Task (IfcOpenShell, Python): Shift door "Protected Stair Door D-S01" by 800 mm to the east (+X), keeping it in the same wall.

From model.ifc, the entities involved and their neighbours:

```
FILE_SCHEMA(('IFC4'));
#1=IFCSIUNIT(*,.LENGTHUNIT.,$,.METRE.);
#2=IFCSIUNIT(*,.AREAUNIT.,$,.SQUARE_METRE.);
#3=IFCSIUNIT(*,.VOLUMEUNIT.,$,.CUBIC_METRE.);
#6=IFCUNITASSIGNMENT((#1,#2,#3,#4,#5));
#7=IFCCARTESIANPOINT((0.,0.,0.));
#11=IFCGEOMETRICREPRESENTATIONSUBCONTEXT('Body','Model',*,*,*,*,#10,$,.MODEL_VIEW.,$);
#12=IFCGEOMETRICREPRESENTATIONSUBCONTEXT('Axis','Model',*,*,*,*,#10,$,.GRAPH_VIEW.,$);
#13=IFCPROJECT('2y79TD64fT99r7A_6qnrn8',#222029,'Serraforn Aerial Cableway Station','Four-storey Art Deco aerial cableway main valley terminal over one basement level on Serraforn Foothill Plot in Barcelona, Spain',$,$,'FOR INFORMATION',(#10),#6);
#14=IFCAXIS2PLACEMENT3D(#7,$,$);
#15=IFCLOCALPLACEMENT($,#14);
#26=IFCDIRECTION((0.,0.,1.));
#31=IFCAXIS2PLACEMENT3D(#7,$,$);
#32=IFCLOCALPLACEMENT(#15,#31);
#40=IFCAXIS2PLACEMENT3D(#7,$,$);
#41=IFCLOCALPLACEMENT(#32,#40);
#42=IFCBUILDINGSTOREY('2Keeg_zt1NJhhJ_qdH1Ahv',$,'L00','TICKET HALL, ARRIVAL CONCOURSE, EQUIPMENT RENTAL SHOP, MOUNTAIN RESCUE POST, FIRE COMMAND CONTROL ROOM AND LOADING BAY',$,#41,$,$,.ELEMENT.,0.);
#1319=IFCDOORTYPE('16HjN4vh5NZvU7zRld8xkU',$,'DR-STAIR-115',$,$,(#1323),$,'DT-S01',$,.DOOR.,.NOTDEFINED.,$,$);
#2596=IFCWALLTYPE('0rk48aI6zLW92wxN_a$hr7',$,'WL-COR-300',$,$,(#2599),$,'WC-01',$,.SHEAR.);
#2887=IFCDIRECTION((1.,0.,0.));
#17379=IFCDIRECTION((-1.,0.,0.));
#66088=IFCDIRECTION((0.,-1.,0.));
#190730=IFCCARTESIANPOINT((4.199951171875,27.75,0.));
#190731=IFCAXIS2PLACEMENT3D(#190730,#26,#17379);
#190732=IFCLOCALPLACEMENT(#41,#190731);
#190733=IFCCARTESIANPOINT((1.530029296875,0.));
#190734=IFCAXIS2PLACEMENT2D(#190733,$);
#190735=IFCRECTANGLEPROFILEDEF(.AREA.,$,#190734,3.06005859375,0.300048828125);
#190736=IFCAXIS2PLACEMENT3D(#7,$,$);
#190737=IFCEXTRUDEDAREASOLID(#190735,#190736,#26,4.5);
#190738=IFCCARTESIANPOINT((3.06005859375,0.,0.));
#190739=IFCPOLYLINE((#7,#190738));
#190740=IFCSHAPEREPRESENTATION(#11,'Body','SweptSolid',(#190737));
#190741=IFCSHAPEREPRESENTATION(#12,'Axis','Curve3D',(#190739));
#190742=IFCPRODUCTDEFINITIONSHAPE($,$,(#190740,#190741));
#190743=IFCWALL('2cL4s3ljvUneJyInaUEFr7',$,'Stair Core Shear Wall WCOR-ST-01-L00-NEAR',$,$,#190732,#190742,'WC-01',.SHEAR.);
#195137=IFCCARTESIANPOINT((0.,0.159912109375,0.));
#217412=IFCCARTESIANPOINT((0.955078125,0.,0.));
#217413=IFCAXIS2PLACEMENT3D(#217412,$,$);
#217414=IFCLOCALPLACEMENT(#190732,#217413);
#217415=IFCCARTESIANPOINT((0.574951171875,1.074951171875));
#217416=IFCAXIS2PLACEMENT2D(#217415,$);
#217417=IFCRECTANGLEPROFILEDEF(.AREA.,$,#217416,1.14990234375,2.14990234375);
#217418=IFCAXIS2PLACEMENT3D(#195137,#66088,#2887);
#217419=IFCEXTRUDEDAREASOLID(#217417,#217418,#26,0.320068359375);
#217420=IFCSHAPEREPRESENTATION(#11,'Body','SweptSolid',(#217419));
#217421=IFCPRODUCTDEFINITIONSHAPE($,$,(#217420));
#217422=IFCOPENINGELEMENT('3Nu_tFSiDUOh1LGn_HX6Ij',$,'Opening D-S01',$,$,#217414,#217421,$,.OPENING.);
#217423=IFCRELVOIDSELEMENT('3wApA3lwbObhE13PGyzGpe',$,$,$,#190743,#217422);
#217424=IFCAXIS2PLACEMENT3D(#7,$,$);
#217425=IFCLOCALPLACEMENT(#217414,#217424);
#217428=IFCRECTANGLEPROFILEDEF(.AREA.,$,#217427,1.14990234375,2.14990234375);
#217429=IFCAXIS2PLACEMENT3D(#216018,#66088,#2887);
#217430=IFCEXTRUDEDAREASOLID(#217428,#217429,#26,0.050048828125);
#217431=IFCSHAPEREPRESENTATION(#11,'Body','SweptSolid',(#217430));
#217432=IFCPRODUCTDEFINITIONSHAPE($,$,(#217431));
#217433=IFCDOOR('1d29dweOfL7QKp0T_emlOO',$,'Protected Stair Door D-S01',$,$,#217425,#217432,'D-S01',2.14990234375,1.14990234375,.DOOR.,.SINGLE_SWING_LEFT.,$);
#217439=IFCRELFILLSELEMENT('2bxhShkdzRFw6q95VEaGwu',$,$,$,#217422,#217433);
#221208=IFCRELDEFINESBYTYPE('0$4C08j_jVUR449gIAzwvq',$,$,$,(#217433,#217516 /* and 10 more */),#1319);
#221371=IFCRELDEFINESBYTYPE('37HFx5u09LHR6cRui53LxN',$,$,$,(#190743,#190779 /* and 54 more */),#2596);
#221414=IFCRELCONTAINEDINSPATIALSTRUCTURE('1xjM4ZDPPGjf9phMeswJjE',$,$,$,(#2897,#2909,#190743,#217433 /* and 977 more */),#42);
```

```python
import ifcopenshell
import ifcopenshell.api.geometry
import ifcopenshell.util.placement
import ifcopenshell.util.unit

model = ifcopenshell.open("model.ifc")
unit_scale = ifcopenshell.util.unit.calculate_unit_scale(model)

door = model.by_guid("1d29dweOfL7QKp0T_emlOO")
opening = door.FillsVoids[0].RelatingOpeningElement
wall = opening.VoidsElements[0].RelatingBuildingElement

wall_matrix = ifcopenshell.util.placement.get_local_placement(wall.ObjectPlacement)
shift = wall_matrix[:3, 0] * -0.8 / unit_scale
before = ifcopenshell.util.placement.get_local_placement(door.ObjectPlacement)[:3, 3].copy()

# The door is placed relative to its opening, so it follows when the opening moves.
matrix = ifcopenshell.util.placement.get_local_placement(opening.ObjectPlacement)
matrix[:3, 3] += shift
ifcopenshell.api.geometry.edit_object_placement(
    model, product=opening, matrix=matrix, is_si=False, should_transform_children=True
)

after = ifcopenshell.util.placement.get_local_placement(door.ObjectPlacement)[:3, 3]
print("door moved by", (after - before).round(3) + 0.0)

model.write("model-out.ifc")
```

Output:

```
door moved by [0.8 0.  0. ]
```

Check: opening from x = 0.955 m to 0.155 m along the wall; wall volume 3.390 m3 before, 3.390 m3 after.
